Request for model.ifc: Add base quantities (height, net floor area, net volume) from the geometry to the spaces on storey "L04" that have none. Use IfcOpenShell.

First a look at what the model holds.

```python
import ifcopenshell
import ifcopenshell.util.element
import ifcopenshell.util.unit

model = ifcopenshell.open("model.ifc")
print(model.schema)
for unit_type in ("LENGTHUNIT", "AREAUNIT", "VOLUMEUNIT"):
    print(unit_type, ifcopenshell.util.unit.calculate_unit_scale(model, unit_type))
storey = next(s for s in model.by_type("IfcBuildingStorey") if s.Name == "L04")
spaces = [e for e in ifcopenshell.util.element.get_decomposition(storey) if e.is_a("IfcSpace")]
for e in sorted(spaces, key=lambda e: e.id()):
    print(e.id(), e.is_a(), e.Name, list(ifcopenshell.util.element.get_psets(e, qtos_only=True)), sep=" | ")
```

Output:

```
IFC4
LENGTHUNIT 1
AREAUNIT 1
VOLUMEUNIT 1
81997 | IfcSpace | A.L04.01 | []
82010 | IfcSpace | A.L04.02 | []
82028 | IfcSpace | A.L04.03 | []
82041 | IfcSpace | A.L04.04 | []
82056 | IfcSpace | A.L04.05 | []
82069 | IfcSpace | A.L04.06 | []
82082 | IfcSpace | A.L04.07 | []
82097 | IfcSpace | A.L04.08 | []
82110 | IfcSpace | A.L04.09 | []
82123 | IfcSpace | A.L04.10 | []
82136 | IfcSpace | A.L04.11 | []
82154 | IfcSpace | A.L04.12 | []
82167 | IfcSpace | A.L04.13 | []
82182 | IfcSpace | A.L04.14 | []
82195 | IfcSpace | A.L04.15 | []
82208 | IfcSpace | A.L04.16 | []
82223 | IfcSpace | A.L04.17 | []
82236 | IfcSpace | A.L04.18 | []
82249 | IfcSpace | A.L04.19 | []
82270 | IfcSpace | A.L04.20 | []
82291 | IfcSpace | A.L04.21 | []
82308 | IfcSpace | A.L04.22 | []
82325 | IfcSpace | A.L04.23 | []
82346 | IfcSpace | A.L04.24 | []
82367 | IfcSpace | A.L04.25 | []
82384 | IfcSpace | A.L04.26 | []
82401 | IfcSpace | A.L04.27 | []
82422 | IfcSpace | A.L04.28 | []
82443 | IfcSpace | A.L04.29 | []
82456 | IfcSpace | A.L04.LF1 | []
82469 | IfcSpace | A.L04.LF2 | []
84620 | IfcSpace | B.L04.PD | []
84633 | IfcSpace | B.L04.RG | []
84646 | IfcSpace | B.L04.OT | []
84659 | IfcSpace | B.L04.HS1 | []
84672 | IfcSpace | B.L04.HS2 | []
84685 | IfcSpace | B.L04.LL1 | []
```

```python
import ifcopenshell
import ifcopenshell.api.pset
import ifcopenshell.geom
import ifcopenshell.util.element
import ifcopenshell.util.shape
import ifcopenshell.util.unit

model = ifcopenshell.open("model.ifc")
unit_scale = ifcopenshell.util.unit.calculate_unit_scale(model)
area_scale = ifcopenshell.util.unit.calculate_unit_scale(model, "AREAUNIT")
volume_scale = ifcopenshell.util.unit.calculate_unit_scale(model, "VOLUMEUNIT")
settings = ifcopenshell.geom.settings()

storey = next(s for s in model.by_type("IfcBuildingStorey") if s.Name == "L04")
spaces = [e for e in ifcopenshell.util.element.get_decomposition(storey) if e.is_a("IfcSpace")]

for e in sorted(spaces, key=lambda e: e.id()):
    if ifcopenshell.util.element.get_psets(e, qtos_only=True, should_inherit=False):
        continue
    # Geometry comes back in metres, in the element's own axes.
    shape = ifcopenshell.geom.create_shape(settings, e)
    values = {
        "Height": ifcopenshell.util.shape.get_z(shape.geometry) / unit_scale,
        "NetFloorArea": ifcopenshell.util.shape.get_footprint_area(shape.geometry) / area_scale,
        "NetVolume": ifcopenshell.util.shape.get_volume(shape.geometry) / volume_scale,
    }
    qto = ifcopenshell.api.pset.add_qto(model, product=e, name="Qto_SpaceBaseQuantities")
    ifcopenshell.api.pset.edit_qto(model, qto=qto, properties=values)
    print(e.id(), {k: round(v, 3) for k, v in values.items()})

model.write("model-out.ifc")
```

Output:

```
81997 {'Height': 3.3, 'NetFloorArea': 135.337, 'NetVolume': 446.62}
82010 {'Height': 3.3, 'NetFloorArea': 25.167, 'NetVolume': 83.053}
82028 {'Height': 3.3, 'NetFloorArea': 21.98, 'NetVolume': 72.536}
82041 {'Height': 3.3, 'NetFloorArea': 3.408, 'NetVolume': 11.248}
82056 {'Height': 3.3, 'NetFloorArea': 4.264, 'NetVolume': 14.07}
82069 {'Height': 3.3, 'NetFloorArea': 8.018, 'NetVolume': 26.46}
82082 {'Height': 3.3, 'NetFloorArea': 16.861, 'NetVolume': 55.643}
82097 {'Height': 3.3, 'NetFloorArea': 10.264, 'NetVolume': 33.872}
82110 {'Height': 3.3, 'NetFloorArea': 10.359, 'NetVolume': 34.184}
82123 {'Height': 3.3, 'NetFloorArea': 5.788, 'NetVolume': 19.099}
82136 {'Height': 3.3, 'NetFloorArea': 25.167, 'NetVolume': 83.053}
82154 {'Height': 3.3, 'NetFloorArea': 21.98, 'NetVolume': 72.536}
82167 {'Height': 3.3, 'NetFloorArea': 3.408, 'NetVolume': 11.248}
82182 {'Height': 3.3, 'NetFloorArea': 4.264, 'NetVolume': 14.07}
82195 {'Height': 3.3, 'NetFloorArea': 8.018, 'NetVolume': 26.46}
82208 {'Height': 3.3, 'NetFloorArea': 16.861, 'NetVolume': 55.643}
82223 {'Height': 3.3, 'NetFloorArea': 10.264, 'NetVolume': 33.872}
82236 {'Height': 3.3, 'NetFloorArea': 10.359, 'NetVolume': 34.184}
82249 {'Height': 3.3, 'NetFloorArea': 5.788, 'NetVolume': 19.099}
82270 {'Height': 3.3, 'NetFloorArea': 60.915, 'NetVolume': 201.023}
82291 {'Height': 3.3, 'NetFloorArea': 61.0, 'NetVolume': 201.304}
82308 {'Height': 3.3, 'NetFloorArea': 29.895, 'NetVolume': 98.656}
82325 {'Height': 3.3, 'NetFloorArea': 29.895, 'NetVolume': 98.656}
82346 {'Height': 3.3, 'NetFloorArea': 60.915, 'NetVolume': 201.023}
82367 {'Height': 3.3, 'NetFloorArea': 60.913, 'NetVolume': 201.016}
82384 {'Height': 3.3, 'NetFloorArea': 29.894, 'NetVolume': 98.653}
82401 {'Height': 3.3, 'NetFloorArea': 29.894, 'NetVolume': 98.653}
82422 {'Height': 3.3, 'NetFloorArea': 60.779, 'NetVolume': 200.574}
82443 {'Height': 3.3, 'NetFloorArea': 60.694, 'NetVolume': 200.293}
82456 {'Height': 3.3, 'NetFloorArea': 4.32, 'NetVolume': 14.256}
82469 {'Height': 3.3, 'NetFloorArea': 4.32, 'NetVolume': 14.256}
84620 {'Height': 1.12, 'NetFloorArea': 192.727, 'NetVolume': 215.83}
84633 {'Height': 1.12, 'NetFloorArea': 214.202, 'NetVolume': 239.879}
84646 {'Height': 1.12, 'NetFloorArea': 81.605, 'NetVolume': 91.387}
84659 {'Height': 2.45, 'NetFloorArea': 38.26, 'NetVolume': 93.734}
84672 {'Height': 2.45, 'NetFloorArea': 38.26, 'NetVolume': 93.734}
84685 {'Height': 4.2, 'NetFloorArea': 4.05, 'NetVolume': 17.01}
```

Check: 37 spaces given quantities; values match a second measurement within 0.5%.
